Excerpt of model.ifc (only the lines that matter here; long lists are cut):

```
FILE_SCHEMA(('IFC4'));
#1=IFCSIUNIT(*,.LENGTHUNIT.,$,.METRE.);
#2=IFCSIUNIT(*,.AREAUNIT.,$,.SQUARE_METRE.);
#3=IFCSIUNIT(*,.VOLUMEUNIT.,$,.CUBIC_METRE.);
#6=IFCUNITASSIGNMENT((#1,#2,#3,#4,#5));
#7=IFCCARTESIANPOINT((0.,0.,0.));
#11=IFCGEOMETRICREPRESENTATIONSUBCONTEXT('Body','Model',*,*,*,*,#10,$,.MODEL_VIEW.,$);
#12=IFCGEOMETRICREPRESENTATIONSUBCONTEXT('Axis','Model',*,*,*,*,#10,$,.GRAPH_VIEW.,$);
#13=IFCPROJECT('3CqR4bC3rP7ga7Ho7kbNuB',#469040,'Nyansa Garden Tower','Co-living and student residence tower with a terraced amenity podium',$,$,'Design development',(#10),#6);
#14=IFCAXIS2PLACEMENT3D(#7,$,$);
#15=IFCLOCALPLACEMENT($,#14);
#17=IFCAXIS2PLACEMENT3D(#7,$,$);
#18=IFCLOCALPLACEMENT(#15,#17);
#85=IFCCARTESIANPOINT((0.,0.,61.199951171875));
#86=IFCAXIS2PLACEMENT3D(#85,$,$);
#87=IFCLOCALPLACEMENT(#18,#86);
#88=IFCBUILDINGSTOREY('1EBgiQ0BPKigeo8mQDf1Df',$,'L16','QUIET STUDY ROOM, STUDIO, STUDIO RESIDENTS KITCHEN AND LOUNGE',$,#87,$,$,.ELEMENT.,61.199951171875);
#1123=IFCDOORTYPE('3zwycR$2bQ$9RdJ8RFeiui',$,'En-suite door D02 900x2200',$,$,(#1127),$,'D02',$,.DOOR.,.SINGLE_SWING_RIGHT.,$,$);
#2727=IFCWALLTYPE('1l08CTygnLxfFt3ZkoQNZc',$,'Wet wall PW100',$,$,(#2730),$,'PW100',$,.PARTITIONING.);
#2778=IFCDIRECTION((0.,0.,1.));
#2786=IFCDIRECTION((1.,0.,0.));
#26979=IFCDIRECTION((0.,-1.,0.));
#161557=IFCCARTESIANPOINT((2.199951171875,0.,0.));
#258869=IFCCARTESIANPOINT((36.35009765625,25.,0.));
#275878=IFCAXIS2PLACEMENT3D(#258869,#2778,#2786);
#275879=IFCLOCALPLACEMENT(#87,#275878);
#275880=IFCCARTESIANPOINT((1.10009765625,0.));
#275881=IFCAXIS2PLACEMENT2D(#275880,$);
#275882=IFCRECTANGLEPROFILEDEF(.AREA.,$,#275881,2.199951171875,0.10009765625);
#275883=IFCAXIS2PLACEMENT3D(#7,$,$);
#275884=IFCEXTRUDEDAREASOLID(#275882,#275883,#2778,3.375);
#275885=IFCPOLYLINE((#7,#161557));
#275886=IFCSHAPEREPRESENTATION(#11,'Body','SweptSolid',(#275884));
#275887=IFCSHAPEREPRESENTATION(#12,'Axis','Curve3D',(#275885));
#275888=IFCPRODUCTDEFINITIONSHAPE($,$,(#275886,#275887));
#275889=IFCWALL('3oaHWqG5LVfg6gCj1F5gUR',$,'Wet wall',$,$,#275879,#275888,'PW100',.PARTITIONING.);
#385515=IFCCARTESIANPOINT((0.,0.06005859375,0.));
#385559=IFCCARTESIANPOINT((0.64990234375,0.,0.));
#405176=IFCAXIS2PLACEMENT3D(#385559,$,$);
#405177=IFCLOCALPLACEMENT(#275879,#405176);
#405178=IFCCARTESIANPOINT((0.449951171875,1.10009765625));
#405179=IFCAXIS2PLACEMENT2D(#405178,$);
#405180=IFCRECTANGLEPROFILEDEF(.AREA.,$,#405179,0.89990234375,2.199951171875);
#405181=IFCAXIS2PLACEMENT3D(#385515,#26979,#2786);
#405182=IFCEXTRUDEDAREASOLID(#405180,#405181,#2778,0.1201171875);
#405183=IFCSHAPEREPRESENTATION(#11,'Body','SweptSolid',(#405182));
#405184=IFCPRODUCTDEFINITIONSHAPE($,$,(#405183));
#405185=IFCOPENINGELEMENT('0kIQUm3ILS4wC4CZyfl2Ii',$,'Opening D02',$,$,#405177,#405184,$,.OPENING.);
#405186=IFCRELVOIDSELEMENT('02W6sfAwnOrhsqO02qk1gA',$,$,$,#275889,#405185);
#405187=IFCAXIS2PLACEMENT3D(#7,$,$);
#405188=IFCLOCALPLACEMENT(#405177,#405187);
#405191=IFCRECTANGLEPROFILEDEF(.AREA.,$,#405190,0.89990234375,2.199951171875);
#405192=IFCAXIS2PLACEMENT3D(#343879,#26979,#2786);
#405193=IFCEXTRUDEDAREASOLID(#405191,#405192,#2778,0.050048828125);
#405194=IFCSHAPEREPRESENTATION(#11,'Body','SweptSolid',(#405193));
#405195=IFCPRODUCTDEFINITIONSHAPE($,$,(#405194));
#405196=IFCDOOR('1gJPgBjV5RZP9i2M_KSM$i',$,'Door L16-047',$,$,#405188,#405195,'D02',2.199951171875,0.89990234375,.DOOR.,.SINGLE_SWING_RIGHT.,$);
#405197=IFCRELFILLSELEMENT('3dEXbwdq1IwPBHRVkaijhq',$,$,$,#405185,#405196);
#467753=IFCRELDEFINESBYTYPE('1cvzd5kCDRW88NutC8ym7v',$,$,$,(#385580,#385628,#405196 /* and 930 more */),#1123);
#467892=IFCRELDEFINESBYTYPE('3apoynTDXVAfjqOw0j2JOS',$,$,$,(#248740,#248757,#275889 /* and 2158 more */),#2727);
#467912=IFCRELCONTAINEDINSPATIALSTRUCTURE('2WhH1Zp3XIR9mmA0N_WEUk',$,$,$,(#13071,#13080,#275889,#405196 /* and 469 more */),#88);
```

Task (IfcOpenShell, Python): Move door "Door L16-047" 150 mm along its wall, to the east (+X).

```python
import ifcopenshell
import ifcopenshell.api.geometry
import ifcopenshell.util.placement
import ifcopenshell.util.unit

model = ifcopenshell.open("model.ifc")
unit_scale = ifcopenshell.util.unit.calculate_unit_scale(model)

door = model.by_guid("1gJPgBjV5RZP9i2M_KSM$i")
opening = door.FillsVoids[0].RelatingOpeningElement
wall = opening.VoidsElements[0].RelatingBuildingElement

wall_matrix = ifcopenshell.util.placement.get_local_placement(wall.ObjectPlacement)
shift = wall_matrix[:3, 0] * 0.15 / unit_scale
before = ifcopenshell.util.placement.get_local_placement(door.ObjectPlacement)[:3, 3].copy()

# The door is placed relative to its opening, so it follows when the opening moves.
matrix = ifcopenshell.util.placement.get_local_placement(opening.ObjectPlacement)
matrix[:3, 3] += shift
ifcopenshell.api.geometry.edit_object_placement(
    model, product=opening, matrix=matrix, is_si=False, should_transform_children=True
)

after = ifcopenshell.util.placement.get_local_placement(door.ObjectPlacement)[:3, 3]
print("door moved by", (after - before).round(3) + 0.0)

model.write("model_rev.ifc")
```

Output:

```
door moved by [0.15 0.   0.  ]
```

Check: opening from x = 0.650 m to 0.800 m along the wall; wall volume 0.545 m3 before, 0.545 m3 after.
